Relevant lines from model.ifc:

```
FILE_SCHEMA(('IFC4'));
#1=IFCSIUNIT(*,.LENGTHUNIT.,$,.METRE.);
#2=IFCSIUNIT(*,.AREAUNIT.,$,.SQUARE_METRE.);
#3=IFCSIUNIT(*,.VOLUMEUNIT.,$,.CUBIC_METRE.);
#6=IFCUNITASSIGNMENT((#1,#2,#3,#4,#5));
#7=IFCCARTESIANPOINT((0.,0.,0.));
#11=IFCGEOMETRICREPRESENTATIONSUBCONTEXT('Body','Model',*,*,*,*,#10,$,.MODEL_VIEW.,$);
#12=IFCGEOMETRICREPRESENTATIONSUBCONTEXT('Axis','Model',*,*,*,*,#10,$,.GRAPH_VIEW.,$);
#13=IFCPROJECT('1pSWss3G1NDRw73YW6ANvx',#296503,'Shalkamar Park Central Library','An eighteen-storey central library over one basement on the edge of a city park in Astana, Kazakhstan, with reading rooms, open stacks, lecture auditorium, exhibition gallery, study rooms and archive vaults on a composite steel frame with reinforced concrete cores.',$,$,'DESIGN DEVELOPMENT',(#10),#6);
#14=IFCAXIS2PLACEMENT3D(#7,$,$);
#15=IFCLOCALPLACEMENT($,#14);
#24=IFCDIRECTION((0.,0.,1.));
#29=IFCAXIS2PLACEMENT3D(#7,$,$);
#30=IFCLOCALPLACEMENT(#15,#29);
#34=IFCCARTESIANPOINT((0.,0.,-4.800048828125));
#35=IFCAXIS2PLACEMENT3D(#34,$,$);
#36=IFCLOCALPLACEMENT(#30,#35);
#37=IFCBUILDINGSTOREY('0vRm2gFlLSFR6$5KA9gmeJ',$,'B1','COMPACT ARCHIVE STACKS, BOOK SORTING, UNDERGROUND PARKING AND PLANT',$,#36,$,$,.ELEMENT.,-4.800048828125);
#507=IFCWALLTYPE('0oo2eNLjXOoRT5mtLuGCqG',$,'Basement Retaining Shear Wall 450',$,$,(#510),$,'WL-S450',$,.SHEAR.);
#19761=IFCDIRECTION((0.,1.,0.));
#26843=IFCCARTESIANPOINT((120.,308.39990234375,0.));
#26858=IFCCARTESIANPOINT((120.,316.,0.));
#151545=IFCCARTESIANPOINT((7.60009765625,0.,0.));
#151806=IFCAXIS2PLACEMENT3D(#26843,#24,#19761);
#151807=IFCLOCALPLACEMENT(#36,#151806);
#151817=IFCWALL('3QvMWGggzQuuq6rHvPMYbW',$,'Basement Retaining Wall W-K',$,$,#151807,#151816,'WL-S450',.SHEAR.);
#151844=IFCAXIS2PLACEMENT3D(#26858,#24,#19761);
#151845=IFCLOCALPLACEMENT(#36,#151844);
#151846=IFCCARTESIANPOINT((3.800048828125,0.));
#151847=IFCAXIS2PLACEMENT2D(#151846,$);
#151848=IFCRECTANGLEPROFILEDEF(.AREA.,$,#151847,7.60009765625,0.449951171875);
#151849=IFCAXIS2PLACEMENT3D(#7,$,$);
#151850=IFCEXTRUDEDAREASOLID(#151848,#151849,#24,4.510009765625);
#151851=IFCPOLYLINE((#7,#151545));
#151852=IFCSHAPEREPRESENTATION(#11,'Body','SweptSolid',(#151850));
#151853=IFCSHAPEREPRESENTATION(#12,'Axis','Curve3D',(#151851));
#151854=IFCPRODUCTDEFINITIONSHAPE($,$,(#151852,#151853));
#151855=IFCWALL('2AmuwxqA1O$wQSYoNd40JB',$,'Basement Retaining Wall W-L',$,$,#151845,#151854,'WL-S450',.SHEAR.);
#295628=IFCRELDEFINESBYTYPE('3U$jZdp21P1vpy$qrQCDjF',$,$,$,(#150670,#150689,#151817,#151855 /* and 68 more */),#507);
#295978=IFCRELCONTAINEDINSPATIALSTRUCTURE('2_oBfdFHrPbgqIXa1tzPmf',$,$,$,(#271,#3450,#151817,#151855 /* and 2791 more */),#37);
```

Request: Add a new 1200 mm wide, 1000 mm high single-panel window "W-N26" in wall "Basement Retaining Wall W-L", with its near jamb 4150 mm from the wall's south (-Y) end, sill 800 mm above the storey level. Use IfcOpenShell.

```python
import numpy as np
import ifcopenshell
import ifcopenshell.api.feature
import ifcopenshell.api.geometry
import ifcopenshell.api.root
import ifcopenshell.api.spatial
import ifcopenshell.geom
import ifcopenshell.util.element
import ifcopenshell.util.placement
import ifcopenshell.util.representation
import ifcopenshell.util.shape
import ifcopenshell.util.unit

model = ifcopenshell.open("model.ifc")
unit_scale = ifcopenshell.util.unit.calculate_unit_scale(model)
settings = ifcopenshell.geom.settings()


def volume(element):
    """Net volume in cubic metres, openings subtracted."""
    shape = ifcopenshell.geom.create_shape(settings, element)
    return ifcopenshell.util.shape.get_volume(shape.geometry)


wall = model.by_guid("2AmuwxqA1O$wQSYoNd40JB")
storey = ifcopenshell.util.element.get_container(wall, ifc_class="IfcBuildingStorey")
context = ifcopenshell.util.representation.get_context(model, "Model", "Body", "MODEL_VIEW")
before = volume(wall)

width, height, from_end, sill = 1.2, 1, 4.15, 0.8  # metres

# The wall runs along its own X axis, and the end named is its -X end.
wall_shape = ifcopenshell.geom.create_shape(settings, wall)
x, y, z = ifcopenshell.util.shape.get_vertices(wall_shape.geometry).T
start = x.min() + from_end
face, thickness = float(y.min()), float(y.max() - y.min())
wall_matrix = ifcopenshell.util.placement.get_local_placement(wall.ObjectPlacement)
level = ifcopenshell.util.placement.get_local_placement(storey.ObjectPlacement)[2, 3]


def in_wall(x, y):
    """Placement at x, y metres in the wall's axes, at sill height."""
    matrix = wall_matrix.copy()
    matrix[:, 3] = wall_matrix @ np.array([x / unit_scale, y / unit_scale, 0.0, 1.0])
    matrix[2, 3] = level + sill / unit_scale
    return matrix


# Opening: a box that overshoots both wall faces by 50 mm.
opening = ifcopenshell.api.root.create_entity(model, ifc_class="IfcOpeningElement", predefined_type="OPENING")
box = ifcopenshell.api.geometry.add_wall_representation(
    model, context=context, length=width, height=height, thickness=thickness + 0.1
)
ifcopenshell.api.geometry.assign_representation(model, product=opening, representation=box)
ifcopenshell.api.geometry.edit_object_placement(model, product=opening, matrix=in_wall(start, face - 0.05), is_si=False)
ifcopenshell.api.feature.add_feature(model, feature=opening, element=wall)

window = ifcopenshell.api.root.create_entity(model, ifc_class="IfcWindow", name="W-N26", predefined_type="WINDOW")
window.OverallWidth, window.OverallHeight = width / unit_scale, height / unit_scale
window.PartitioningType = "SINGLE_PANEL"
body = ifcopenshell.api.geometry.add_window_representation(
    model,
    context=context,
    overall_width=window.OverallWidth,
    overall_height=window.OverallHeight,
    partition_type="SINGLE_PANEL",
)
ifcopenshell.api.geometry.assign_representation(model, product=window, representation=body)
ifcopenshell.api.spatial.assign_container(model, products=[window], relating_structure=storey)
ifcopenshell.api.feature.add_filling(model, opening=opening, element=window)

# Centre the window in the wall's thickness.
ifcopenshell.api.geometry.edit_object_placement(model, product=window, matrix=in_wall(start, face), is_si=False)
window_shape = ifcopenshell.geom.create_shape(settings, window)
depth = ifcopenshell.util.shape.get_vertices(window_shape.geometry)[:, 1]
offset = face + thickness / 2 - (depth.min() + depth.max()) / 2
ifcopenshell.api.geometry.edit_object_placement(model, product=window, matrix=in_wall(start, offset), is_si=False)

after = volume(wall)

print(f"wall volume {before:.3f} -> {after:.3f} m3")

model.write("model-out.ifc")
```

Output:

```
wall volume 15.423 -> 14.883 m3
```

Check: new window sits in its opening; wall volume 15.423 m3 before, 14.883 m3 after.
